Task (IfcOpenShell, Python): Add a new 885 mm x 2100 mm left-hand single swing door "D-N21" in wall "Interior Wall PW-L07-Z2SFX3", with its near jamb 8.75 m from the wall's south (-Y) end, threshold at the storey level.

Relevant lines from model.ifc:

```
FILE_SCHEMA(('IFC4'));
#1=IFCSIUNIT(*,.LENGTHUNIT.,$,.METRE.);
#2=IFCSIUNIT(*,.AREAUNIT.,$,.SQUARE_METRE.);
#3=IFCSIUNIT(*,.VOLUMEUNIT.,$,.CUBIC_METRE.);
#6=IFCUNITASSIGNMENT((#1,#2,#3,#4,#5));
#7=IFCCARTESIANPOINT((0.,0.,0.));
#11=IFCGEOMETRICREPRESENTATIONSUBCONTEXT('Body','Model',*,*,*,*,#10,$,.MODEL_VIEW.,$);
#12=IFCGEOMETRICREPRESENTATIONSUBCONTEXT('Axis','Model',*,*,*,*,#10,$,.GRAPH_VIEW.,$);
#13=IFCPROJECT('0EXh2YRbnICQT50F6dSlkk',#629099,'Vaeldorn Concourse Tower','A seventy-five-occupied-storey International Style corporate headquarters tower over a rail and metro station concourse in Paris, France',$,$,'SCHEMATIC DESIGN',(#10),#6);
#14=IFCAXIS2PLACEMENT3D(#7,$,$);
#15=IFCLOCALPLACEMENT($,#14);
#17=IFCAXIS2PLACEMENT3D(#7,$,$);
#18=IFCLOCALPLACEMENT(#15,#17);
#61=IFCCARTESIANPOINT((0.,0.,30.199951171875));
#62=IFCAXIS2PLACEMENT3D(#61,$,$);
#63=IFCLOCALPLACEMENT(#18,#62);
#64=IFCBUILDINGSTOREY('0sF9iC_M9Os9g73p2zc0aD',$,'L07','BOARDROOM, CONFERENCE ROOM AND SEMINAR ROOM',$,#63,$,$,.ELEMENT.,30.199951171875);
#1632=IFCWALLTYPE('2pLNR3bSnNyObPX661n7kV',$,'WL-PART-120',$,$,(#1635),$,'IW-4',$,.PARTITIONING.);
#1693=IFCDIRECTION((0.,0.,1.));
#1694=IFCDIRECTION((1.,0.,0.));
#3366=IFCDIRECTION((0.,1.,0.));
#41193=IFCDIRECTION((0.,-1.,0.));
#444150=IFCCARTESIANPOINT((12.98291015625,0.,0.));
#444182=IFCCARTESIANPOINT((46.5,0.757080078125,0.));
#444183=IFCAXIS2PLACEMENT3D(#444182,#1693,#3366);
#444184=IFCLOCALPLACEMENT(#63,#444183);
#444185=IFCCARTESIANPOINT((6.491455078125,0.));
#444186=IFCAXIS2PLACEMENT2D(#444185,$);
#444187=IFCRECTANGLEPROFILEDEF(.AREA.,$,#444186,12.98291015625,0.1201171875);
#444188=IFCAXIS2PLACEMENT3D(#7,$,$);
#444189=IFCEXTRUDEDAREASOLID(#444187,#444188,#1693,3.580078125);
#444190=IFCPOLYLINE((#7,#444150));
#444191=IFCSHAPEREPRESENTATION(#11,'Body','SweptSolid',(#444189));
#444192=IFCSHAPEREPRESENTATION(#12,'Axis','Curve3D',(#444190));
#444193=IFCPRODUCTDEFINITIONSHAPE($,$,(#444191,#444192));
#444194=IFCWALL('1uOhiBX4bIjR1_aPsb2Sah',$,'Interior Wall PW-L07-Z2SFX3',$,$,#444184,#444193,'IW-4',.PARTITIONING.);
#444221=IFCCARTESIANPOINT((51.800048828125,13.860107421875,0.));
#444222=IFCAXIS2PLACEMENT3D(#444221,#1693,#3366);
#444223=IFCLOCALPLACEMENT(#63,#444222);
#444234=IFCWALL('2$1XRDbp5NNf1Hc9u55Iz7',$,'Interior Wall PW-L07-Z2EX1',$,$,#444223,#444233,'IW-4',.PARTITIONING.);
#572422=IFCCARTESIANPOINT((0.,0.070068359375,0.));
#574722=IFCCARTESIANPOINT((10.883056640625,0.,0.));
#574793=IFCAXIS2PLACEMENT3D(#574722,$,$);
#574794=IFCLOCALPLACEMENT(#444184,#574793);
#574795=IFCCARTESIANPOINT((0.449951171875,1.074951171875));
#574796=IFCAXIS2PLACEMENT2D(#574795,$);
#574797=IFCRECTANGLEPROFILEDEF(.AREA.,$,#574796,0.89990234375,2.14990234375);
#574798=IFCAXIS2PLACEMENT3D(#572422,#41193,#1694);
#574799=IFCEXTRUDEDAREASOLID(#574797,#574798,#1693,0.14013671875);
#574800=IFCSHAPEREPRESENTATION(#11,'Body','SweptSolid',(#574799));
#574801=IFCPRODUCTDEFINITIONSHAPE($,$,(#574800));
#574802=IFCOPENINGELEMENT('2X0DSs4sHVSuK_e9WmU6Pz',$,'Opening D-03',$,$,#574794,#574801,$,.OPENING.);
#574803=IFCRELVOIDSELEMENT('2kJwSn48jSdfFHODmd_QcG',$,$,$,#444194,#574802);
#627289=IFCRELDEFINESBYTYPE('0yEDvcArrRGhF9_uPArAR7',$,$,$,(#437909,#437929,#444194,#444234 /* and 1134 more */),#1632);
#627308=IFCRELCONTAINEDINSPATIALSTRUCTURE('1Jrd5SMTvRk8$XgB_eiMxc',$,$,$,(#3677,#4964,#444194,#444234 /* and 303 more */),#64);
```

```python
import numpy as np
import ifcopenshell
import ifcopenshell.api.feature
import ifcopenshell.api.geometry
import ifcopenshell.api.root
import ifcopenshell.api.spatial
import ifcopenshell.geom
import ifcopenshell.util.element
import ifcopenshell.util.placement
import ifcopenshell.util.representation
import ifcopenshell.util.shape
import ifcopenshell.util.unit

model = ifcopenshell.open("model.ifc")
unit_scale = ifcopenshell.util.unit.calculate_unit_scale(model)
settings = ifcopenshell.geom.settings()


def volume(element):
    """Net volume in cubic metres, openings subtracted."""
    shape = ifcopenshell.geom.create_shape(settings, element)
    return ifcopenshell.util.shape.get_volume(shape.geometry)


wall = model.by_guid("1uOhiBX4bIjR1_aPsb2Sah")
storey = ifcopenshell.util.element.get_container(wall, ifc_class="IfcBuildingStorey")
context = ifcopenshell.util.representation.get_context(model, "Model", "Body", "MODEL_VIEW")
before = volume(wall)

width, height, from_end, sill = 0.885, 2.1, 8.75, 0.0  # metres

# The wall runs along its own X axis, and the end named is its -X end.
wall_shape = ifcopenshell.geom.create_shape(settings, wall)
x, y, z = ifcopenshell.util.shape.get_vertices(wall_shape.geometry).T
start = x.min() + from_end
face, thickness = float(y.min()), float(y.max() - y.min())
wall_matrix = ifcopenshell.util.placement.get_local_placement(wall.ObjectPlacement)
level = ifcopenshell.util.placement.get_local_placement(storey.ObjectPlacement)[2, 3]


def in_wall(x, y):
    """Placement at x, y metres in the wall's axes, at sill height."""
    matrix = wall_matrix.copy()
    matrix[:, 3] = wall_matrix @ np.array([x / unit_scale, y / unit_scale, 0.0, 1.0])
    matrix[2, 3] = level + sill / unit_scale
    return matrix


# Opening: a box that overshoots both wall faces by 50 mm.
opening = ifcopenshell.api.root.create_entity(model, ifc_class="IfcOpeningElement", predefined_type="OPENING")
box = ifcopenshell.api.geometry.add_wall_representation(
    model, context=context, length=width, height=height, thickness=thickness + 0.1
)
ifcopenshell.api.geometry.assign_representation(model, product=opening, representation=box)
ifcopenshell.api.geometry.edit_object_placement(model, product=opening, matrix=in_wall(start, face - 0.05), is_si=False)
ifcopenshell.api.feature.add_feature(model, feature=opening, element=wall)

door = ifcopenshell.api.root.create_entity(model, ifc_class="IfcDoor", name="D-N21", predefined_type="DOOR")
door.OverallWidth, door.OverallHeight = width / unit_scale, height / unit_scale
door.OperationType = "SINGLE_SWING_LEFT"
body = ifcopenshell.api.geometry.add_door_representation(
    model,
    context=context,
    overall_width=door.OverallWidth,
    overall_height=door.OverallHeight,
    operation_type="SINGLE_SWING_LEFT",
    lining_properties={"LiningDepth": thickness / unit_scale, "ThresholdDepth": thickness / unit_scale},
)
ifcopenshell.api.geometry.assign_representation(model, product=door, representation=body)
ifcopenshell.api.spatial.assign_container(model, products=[door], relating_structure=storey)
ifcopenshell.api.feature.add_filling(model, opening=opening, element=door)

# The lining spans the wall, so the door starts at the wall face.
ifcopenshell.api.geometry.edit_object_placement(model, product=door, matrix=in_wall(start, face), is_si=False)

after = volume(wall)

print(f"wall volume {before:.3f} -> {after:.3f} m3")

model.write("model_updated.ifc")
```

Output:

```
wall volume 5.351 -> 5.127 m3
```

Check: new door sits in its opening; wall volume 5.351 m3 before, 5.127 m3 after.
